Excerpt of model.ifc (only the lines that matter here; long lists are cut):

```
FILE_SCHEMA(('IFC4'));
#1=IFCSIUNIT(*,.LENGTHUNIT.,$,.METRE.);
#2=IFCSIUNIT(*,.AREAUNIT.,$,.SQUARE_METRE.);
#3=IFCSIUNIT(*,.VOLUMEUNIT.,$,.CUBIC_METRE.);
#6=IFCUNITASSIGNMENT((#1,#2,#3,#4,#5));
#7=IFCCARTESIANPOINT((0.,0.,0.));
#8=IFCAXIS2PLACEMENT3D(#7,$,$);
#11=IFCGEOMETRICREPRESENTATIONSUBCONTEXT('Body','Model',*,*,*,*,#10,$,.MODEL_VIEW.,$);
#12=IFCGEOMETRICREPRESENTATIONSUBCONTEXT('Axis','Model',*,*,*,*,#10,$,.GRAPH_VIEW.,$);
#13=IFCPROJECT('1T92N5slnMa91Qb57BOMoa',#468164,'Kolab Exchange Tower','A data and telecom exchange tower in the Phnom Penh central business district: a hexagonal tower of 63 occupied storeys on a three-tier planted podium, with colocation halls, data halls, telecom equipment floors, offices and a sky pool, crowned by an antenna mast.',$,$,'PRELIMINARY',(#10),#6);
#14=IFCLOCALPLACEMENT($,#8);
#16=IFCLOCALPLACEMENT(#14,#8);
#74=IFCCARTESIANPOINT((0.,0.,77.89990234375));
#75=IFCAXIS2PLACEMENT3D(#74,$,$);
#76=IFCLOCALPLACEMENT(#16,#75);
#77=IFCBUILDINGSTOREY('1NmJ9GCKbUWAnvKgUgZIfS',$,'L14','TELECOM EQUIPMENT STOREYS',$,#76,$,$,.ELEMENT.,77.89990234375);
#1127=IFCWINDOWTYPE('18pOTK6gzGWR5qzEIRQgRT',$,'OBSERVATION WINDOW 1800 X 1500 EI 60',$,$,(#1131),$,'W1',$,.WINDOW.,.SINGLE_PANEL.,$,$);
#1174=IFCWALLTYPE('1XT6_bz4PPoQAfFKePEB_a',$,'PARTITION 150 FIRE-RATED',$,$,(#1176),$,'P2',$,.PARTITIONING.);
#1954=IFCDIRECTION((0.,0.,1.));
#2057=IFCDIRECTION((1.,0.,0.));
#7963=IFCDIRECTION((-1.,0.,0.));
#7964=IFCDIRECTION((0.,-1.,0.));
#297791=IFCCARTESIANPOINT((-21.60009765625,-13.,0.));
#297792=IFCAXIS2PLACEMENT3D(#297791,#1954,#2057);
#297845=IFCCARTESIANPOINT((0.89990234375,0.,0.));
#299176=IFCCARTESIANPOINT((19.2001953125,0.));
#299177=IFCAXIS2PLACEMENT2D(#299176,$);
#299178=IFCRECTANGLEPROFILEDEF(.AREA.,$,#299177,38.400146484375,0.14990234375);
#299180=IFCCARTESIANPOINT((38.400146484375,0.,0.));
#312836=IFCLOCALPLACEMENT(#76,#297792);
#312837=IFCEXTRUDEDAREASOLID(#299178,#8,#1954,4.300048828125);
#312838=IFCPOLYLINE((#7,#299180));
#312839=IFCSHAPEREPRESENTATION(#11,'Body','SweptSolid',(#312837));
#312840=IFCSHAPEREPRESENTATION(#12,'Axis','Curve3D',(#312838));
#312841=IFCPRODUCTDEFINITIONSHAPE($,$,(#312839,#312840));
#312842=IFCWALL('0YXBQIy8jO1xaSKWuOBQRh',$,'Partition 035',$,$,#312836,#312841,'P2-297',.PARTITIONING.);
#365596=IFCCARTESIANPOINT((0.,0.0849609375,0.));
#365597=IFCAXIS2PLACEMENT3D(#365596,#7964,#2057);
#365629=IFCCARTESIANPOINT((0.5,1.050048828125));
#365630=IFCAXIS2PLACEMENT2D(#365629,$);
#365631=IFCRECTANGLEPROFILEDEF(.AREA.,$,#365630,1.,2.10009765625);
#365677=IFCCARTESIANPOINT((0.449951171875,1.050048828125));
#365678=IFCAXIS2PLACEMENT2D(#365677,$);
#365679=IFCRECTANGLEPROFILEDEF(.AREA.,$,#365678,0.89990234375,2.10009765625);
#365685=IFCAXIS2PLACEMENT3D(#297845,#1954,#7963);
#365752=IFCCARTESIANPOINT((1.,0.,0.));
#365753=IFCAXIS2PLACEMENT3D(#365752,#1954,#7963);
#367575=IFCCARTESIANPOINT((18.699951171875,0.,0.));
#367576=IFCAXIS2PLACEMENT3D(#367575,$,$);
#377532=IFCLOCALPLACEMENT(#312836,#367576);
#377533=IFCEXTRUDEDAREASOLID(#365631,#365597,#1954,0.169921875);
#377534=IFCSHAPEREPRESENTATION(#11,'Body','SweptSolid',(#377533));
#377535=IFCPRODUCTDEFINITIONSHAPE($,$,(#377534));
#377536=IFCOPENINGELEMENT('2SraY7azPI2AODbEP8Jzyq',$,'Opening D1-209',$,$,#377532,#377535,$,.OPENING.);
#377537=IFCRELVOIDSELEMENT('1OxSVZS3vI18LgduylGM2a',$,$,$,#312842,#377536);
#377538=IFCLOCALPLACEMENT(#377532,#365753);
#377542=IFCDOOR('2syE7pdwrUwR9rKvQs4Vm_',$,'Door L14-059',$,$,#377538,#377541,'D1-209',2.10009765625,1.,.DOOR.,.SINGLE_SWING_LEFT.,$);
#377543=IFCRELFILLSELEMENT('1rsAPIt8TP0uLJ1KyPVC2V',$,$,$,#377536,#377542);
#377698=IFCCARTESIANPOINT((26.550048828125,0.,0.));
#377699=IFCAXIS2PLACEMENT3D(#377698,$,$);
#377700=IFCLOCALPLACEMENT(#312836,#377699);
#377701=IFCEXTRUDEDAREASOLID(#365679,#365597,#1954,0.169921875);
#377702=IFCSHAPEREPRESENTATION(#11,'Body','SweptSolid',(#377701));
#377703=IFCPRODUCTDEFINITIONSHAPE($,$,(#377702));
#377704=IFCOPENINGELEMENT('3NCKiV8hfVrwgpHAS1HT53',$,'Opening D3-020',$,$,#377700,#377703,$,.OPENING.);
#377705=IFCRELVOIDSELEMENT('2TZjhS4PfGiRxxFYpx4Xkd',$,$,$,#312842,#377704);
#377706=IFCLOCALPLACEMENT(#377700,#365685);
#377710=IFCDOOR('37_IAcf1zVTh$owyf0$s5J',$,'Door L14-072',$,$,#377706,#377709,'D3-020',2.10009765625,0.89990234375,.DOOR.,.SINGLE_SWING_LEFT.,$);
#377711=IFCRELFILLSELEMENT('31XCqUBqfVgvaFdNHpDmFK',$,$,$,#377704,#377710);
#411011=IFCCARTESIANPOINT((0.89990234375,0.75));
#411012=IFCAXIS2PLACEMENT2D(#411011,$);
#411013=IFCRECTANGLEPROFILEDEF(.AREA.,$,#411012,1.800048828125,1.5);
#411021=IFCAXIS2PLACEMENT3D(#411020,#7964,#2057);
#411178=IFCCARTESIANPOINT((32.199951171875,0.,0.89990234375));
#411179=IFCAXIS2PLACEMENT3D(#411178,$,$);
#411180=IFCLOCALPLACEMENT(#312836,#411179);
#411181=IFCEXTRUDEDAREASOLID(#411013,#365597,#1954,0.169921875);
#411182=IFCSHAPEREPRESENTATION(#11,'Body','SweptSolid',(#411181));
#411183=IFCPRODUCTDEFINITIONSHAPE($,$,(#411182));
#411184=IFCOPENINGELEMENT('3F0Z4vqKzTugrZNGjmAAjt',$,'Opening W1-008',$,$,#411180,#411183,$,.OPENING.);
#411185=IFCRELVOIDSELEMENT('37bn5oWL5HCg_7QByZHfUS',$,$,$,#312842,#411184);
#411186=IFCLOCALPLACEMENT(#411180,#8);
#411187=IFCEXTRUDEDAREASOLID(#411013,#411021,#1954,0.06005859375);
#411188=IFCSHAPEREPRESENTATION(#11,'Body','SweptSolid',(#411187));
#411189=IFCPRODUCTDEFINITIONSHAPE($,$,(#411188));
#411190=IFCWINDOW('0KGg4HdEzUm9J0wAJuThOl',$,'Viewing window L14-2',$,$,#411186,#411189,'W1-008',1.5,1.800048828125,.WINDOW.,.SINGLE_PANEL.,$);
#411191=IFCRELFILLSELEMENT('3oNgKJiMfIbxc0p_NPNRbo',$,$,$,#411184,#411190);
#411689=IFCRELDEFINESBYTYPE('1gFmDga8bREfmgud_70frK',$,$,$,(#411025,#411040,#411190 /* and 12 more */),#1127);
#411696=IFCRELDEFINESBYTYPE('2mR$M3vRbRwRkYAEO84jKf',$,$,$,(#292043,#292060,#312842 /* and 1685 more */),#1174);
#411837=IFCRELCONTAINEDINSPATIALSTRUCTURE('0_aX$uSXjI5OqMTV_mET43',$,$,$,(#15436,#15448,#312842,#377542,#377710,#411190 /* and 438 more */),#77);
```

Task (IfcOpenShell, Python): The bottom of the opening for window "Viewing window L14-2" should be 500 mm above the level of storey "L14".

```python
import numpy as np
import ifcopenshell
import ifcopenshell.api.geometry
import ifcopenshell.geom
import ifcopenshell.util.element
import ifcopenshell.util.placement
import ifcopenshell.util.shape
import ifcopenshell.util.unit

model = ifcopenshell.open("model.ifc")
unit_scale = ifcopenshell.util.unit.calculate_unit_scale(model)

window = model.by_id(411190)
opening = window.FillsVoids[0].RelatingOpeningElement
storey = ifcopenshell.util.element.get_container(window, ifc_class="IfcBuildingStorey")
level = ifcopenshell.util.placement.get_local_placement(storey.ObjectPlacement)[2, 3]

# The opening's origin need not be at the sill, so measure its lowest point.
shape = ifcopenshell.geom.create_shape(ifcopenshell.geom.settings(), opening)
bottom = ifcopenshell.util.shape.get_shape_bottom_elevation(shape, shape.geometry) / unit_scale
dz = level + 0.5 / unit_scale - bottom

shift = np.array([0.0, 0.0, dz])
# The window is placed relative to its opening, so it follows when the opening moves.
matrix = ifcopenshell.util.placement.get_local_placement(opening.ObjectPlacement)
matrix[:3, 3] += shift
ifcopenshell.api.geometry.edit_object_placement(
    model, product=opening, matrix=matrix, is_si=False, should_transform_children=True
)

print(f"moved by {dz * unit_scale:+.3f} m")

model.write("model_v2.ifc")
```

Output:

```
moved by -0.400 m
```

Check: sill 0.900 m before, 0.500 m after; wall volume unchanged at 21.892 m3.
